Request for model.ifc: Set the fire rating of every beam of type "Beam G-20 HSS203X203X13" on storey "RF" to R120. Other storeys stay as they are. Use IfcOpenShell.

First a look at what the model holds.

```python
import ifcopenshell
import ifcopenshell.util.element

model = ifcopenshell.open("model.ifc")
print(model.schema)
storey = next(s for s in model.by_type("IfcBuildingStorey") if s.Name == "RF")
beams = [e for e in ifcopenshell.util.element.get_decomposition(storey) if e.is_a("IfcBeam")]
seen = {}
for e in beams:
    element_type = ifcopenshell.util.element.get_type(e)
    key = (element_type.Name if element_type != e and element_type else None, ifcopenshell.util.element.get_pset(e, "Pset_BeamCommon", "FireRating"))
    seen[key] = seen.get(key, 0) + 1
for (name, value), count in sorted(seen.items(), key=str):
    print(count, "x", name, "|", value)
```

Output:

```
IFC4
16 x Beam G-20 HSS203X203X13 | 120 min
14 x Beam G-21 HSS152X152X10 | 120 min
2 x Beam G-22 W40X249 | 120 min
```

```python
import ifcopenshell
import ifcopenshell.api.pset
import ifcopenshell.util.element

model = ifcopenshell.open("model.ifc")

storey = next(s for s in model.by_type("IfcBuildingStorey") if s.Name == "RF")
beams = [e for e in ifcopenshell.util.element.get_decomposition(storey) if e.is_a("IfcBeam")]

count = 0
for e in beams:
    element_type = ifcopenshell.util.element.get_type(e)
    if element_type in (None, e) or element_type.Name != "Beam G-20 HSS203X203X13":
        continue
    # add_pset returns the element's existing set when there is one.
    pset = ifcopenshell.api.pset.add_pset(model, product=e, name="Pset_BeamCommon")
    ifcopenshell.api.pset.edit_pset(model, pset=pset, properties={"FireRating": "R120"})
    count += 1

print(count, "beams updated")

model.write("model-out.ifc")
```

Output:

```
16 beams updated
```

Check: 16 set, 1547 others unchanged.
